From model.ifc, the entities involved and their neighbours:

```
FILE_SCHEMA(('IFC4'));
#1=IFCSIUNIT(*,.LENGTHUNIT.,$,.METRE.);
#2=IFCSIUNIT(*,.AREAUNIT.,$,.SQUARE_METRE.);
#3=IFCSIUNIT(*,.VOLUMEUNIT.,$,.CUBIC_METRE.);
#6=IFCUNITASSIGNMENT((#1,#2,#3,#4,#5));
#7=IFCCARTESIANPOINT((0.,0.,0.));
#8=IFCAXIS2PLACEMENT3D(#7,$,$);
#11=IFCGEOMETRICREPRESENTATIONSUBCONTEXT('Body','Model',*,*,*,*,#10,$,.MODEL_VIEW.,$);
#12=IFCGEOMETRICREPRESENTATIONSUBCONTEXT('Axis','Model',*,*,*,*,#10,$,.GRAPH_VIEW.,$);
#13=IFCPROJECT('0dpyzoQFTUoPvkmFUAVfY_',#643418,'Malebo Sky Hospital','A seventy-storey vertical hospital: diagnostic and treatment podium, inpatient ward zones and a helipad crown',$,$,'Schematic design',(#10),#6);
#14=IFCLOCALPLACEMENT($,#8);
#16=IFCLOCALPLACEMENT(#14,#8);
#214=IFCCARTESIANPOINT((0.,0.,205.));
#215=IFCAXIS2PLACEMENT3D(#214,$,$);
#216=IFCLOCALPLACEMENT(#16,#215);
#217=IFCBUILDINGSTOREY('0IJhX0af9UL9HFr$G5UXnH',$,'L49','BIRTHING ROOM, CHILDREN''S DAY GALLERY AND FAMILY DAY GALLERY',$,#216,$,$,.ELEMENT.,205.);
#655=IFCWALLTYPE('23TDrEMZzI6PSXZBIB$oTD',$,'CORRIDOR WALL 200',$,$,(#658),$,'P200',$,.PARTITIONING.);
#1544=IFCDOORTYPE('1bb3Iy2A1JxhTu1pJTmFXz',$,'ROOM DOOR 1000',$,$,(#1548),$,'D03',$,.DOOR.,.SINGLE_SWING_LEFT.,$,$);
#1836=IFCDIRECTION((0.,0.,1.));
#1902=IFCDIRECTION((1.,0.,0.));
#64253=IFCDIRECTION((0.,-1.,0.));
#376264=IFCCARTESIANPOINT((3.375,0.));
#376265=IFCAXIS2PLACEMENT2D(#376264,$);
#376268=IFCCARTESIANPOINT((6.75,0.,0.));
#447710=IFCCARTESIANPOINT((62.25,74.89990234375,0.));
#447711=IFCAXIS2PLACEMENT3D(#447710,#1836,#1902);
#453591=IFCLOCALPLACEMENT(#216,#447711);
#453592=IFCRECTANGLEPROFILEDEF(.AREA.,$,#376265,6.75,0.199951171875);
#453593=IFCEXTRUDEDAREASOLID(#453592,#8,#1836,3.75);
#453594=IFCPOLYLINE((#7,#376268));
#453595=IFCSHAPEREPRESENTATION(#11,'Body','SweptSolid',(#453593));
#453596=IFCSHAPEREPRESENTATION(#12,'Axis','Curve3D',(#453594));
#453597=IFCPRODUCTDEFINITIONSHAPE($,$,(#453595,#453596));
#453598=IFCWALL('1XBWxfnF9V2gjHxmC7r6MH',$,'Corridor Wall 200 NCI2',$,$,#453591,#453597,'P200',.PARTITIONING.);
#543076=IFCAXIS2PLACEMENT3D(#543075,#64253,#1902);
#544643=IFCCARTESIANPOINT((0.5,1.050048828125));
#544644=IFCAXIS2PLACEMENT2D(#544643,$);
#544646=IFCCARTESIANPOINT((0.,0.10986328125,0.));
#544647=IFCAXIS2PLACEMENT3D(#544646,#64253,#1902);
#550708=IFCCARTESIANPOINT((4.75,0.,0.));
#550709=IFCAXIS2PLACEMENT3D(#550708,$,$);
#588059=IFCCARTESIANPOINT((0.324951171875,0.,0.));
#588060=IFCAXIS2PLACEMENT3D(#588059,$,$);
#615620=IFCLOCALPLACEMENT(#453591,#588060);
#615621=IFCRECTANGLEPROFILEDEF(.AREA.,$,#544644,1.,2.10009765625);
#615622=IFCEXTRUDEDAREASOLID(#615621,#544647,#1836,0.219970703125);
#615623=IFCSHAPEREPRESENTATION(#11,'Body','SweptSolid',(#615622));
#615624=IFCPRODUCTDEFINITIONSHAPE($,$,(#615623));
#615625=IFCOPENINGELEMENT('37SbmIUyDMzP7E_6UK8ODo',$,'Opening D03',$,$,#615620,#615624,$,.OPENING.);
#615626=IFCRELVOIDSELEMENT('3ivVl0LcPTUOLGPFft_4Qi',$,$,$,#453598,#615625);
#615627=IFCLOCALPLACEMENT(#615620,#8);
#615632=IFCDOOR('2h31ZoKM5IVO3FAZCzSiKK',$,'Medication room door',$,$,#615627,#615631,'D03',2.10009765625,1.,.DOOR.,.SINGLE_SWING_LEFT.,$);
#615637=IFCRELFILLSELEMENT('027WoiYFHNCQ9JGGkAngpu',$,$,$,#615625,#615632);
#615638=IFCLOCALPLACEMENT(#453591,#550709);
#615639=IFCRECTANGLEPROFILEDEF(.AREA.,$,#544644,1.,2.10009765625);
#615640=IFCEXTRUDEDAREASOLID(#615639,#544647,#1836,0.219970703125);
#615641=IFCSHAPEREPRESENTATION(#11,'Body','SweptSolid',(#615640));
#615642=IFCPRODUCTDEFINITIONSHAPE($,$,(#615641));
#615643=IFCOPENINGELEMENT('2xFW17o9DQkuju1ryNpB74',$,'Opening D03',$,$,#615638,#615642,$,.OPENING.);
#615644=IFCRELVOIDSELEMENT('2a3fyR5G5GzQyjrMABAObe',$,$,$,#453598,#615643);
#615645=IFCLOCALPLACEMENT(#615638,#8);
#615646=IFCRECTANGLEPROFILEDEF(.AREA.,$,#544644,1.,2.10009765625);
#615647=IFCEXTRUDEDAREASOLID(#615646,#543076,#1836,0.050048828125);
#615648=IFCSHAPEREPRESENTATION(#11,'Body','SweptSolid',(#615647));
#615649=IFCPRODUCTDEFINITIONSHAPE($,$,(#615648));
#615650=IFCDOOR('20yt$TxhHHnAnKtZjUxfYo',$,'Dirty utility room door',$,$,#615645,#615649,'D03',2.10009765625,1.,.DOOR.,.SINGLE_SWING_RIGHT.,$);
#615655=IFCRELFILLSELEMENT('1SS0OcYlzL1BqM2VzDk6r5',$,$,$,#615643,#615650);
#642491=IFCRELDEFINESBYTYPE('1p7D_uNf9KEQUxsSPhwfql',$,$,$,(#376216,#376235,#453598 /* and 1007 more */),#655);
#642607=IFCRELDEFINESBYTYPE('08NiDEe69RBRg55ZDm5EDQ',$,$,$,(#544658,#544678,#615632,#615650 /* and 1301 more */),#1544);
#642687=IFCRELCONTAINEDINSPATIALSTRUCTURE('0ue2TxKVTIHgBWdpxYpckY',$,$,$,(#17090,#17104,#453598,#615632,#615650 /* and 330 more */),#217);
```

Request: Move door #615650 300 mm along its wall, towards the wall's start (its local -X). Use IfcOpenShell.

```python
import ifcopenshell
import ifcopenshell.api.geometry
import ifcopenshell.util.placement

model = ifcopenshell.open("model.ifc")

door = model.by_guid("20yt$TxhHHnAnKtZjUxfYo")
opening = door.FillsVoids[0].RelatingOpeningElement
wall = opening.VoidsElements[0].RelatingBuildingElement

wall_matrix = ifcopenshell.util.placement.get_local_placement(wall.ObjectPlacement)
shift = wall_matrix[:3, 0] * -0.3
before = ifcopenshell.util.placement.get_local_placement(door.ObjectPlacement)[:3, 3].copy()

# The door is placed relative to its opening, so it follows when the opening moves.
matrix = ifcopenshell.util.placement.get_local_placement(opening.ObjectPlacement)
matrix[:3, 3] += shift
ifcopenshell.api.geometry.edit_object_placement(
    model, product=opening, matrix=matrix, is_si=False, should_transform_children=True
)

after = ifcopenshell.util.placement.get_local_placement(door.ObjectPlacement)[:3, 3]
print("door moved by", (after - before).round(3) + 0.0)

model.write("model_v2.ifc")
```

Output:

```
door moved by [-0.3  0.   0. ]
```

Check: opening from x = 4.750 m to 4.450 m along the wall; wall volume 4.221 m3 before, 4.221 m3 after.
